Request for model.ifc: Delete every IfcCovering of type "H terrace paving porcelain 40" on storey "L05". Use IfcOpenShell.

First a look at what the model holds.

```python
import ifcopenshell
import ifcopenshell.util.element

model = ifcopenshell.open("model.ifc")
print(model.schema)
storey = next(s for s in model.by_type("IfcBuildingStorey") if s.Name == "L05")
coverings = [e for e in ifcopenshell.util.element.get_decomposition(storey) if e.is_a("IfcCovering")]
seen = {}
for e in coverings:
    element_type = ifcopenshell.util.element.get_type(e)
    name = element_type.Name if element_type not in (None, e) else None
    seen[name] = seen.get(name, 0) + 1
for name, count in sorted(seen.items(), key=str):
    print(count, "x", name)
```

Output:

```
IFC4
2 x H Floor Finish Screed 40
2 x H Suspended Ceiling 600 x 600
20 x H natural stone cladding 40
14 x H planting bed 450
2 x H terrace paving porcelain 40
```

```python
import ifcopenshell
import ifcopenshell.api.root
import ifcopenshell.util.element

model = ifcopenshell.open("model.ifc")

storey = next(s for s in model.by_type("IfcBuildingStorey") if s.Name == "L05")
coverings = [e for e in ifcopenshell.util.element.get_decomposition(storey) if e.is_a("IfcCovering")]
targets = [e for e in coverings if (t := ifcopenshell.util.element.get_type(e)) not in (None, e) and t.Name == "H terrace paving porcelain 40"]

for e in targets:
    ifcopenshell.api.root.remove_product(model, product=e)
print(len(targets), "removed")

model.write("model_v2.ifc")
```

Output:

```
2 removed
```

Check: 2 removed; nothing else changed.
